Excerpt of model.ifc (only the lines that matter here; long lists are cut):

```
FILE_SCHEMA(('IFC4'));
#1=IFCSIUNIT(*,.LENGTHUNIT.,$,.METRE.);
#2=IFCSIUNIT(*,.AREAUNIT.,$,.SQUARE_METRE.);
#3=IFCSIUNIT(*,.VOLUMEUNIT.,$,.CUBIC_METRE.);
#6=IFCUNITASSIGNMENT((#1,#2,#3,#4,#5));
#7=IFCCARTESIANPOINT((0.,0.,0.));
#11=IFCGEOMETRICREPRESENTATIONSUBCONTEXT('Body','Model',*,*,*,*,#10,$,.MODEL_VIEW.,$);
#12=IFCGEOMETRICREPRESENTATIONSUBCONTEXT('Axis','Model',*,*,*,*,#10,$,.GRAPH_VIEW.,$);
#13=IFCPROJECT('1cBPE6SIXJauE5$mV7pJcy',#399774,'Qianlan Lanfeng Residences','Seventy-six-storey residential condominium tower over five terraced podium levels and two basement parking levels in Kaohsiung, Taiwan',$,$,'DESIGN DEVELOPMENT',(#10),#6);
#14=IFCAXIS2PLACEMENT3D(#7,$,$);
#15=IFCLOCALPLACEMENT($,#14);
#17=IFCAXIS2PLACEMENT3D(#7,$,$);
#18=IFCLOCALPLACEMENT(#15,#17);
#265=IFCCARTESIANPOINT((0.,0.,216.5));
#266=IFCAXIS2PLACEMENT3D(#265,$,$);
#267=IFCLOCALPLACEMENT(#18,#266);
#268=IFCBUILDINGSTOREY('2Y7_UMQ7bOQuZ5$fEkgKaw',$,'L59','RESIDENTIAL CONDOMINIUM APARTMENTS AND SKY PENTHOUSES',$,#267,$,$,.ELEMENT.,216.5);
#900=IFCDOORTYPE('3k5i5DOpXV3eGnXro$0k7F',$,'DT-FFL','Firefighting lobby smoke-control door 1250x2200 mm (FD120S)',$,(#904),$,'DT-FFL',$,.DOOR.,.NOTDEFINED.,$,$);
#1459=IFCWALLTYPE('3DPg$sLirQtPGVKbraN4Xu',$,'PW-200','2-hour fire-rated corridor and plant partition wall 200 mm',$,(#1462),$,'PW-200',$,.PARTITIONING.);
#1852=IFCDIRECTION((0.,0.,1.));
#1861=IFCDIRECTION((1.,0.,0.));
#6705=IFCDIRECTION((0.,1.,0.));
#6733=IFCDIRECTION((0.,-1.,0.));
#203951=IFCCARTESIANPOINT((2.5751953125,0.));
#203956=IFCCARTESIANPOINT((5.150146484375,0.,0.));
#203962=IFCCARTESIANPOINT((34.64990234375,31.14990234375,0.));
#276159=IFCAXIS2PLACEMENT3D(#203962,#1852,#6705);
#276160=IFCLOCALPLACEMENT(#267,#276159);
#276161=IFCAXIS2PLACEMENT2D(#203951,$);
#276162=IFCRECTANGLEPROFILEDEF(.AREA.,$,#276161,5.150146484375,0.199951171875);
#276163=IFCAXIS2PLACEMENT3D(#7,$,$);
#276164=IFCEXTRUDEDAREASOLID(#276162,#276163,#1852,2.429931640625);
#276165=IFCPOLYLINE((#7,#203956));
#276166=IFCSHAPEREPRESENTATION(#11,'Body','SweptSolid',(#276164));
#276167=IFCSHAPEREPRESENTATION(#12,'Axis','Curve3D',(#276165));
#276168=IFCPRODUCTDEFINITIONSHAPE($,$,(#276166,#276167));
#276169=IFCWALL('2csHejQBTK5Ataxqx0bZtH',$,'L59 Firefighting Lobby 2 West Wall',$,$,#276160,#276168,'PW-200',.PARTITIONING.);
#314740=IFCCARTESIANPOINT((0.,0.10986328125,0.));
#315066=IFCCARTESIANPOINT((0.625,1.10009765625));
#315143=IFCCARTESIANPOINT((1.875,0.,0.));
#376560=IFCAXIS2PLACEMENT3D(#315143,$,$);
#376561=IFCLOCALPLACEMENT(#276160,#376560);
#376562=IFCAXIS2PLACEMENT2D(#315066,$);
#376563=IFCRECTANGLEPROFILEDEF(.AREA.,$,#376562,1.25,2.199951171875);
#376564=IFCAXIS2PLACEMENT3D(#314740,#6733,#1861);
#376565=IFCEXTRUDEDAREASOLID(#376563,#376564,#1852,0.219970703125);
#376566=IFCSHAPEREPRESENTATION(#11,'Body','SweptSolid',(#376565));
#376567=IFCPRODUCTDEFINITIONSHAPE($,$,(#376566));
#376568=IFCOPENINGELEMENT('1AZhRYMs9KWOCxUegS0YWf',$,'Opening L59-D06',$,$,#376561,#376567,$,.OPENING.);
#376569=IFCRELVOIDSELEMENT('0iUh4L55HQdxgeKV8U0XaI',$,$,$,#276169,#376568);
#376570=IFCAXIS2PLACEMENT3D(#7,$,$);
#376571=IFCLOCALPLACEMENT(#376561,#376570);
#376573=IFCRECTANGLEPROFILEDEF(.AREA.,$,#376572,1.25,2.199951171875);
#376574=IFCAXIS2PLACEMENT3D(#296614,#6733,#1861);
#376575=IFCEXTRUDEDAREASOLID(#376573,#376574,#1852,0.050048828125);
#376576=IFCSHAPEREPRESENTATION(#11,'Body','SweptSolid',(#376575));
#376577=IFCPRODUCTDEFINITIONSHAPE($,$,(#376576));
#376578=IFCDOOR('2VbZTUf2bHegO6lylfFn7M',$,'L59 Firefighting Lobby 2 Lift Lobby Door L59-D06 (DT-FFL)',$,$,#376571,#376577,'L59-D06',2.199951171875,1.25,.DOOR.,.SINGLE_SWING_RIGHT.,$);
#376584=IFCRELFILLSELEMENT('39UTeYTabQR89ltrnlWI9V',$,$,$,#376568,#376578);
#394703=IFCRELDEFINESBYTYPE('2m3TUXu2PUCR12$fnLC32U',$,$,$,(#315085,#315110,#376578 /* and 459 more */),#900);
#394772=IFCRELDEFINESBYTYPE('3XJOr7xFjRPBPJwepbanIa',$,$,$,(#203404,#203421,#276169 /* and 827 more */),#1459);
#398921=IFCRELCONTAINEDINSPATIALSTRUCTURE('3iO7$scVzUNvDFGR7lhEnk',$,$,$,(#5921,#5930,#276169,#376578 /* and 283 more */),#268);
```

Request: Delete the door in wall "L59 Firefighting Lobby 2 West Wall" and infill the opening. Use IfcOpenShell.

```python
import ifcopenshell
import ifcopenshell.api.feature
import ifcopenshell.api.root
import ifcopenshell.geom
import ifcopenshell.util.shape

model = ifcopenshell.open("model.ifc")
settings = ifcopenshell.geom.settings()


def volume(element):
    """Net volume in cubic metres, openings subtracted."""
    shape = ifcopenshell.geom.create_shape(settings, element)
    return ifcopenshell.util.shape.get_volume(shape.geometry)


door = model.by_guid("2VbZTUf2bHegO6lylfFn7M")
opening = door.FillsVoids[0].RelatingOpeningElement
wall = opening.VoidsElements[0].RelatingBuildingElement
before = volume(wall)

ifcopenshell.api.root.remove_product(model, product=door)
ifcopenshell.api.feature.remove_feature(model, feature=opening)

after = volume(wall)

print(f"wall volume {before:.3f} -> {after:.3f} m3")

model.write("model_rev.ifc")
```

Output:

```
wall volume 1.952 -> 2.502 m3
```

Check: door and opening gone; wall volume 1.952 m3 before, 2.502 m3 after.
